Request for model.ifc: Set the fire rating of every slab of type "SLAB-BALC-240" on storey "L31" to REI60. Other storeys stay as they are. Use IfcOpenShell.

First a look at what the model holds.

```python
import ifcopenshell
import ifcopenshell.util.element

model = ifcopenshell.open("model.ifc")
print(model.schema)
storey = next(s for s in model.by_type("IfcBuildingStorey") if s.Name == "L31")
slabs = [e for e in ifcopenshell.util.element.get_decomposition(storey) if e.is_a("IfcSlab")]
seen = {}
for e in slabs:
    element_type = ifcopenshell.util.element.get_type(e)
    key = (element_type.Name if element_type != e and element_type else None, ifcopenshell.util.element.get_pset(e, "Pset_SlabCommon", "FireRating"))
    seen[key] = seen.get(key, 0) + 1
for (name, value), count in sorted(seen.items(), key=str):
    print(count, "x", name, "|", value)
```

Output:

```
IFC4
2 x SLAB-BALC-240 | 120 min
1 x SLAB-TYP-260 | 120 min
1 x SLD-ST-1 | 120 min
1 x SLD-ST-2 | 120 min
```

```python
import ifcopenshell
import ifcopenshell.api.pset
import ifcopenshell.util.element

model = ifcopenshell.open("model.ifc")

storey = next(s for s in model.by_type("IfcBuildingStorey") if s.Name == "L31")
slabs = [e for e in ifcopenshell.util.element.get_decomposition(storey) if e.is_a("IfcSlab")]

count = 0
for e in slabs:
    element_type = ifcopenshell.util.element.get_type(e)
    if element_type in (None, e) or element_type.Name != "SLAB-BALC-240":
        continue
    found = ifcopenshell.util.element.get_pset(e, "Pset_SlabCommon", should_inherit=False)
    if found:
        pset = model.by_id(found["id"])
        if len(ifcopenshell.util.element.get_elements_by_pset(pset)) > 1:
            pset = ifcopenshell.api.pset.unshare_pset(model, products=[e], pset=pset)[0]
    else:
        pset = ifcopenshell.api.pset.add_pset(model, product=e, name="Pset_SlabCommon")
    ifcopenshell.api.pset.edit_pset(model, pset=pset, properties={"FireRating": "REI60"})
    count += 1

print(count, "slabs updated")

model.write("model_rev.ifc")
```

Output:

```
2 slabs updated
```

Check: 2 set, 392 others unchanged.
